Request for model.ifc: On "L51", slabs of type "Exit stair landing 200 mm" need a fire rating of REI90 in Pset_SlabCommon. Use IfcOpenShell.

First a look at what the model holds.

```python
import ifcopenshell
import ifcopenshell.util.element

model = ifcopenshell.open("model.ifc")
print(model.schema)
storey = next(s for s in model.by_type("IfcBuildingStorey") if s.Name == "L51")
slabs = [e for e in ifcopenshell.util.element.get_decomposition(storey) if e.is_a("IfcSlab")]
seen = {}
for e in slabs:
    element_type = ifcopenshell.util.element.get_type(e)
    key = (element_type.Name if element_type != e and element_type else None, ifcopenshell.util.element.get_pset(e, "Pset_SlabCommon", "FireRating"))
    seen[key] = seen.get(key, 0) + 1
for (name, value), count in sorted(seen.items(), key=str):
    print(count, "x", name, "|", value)
```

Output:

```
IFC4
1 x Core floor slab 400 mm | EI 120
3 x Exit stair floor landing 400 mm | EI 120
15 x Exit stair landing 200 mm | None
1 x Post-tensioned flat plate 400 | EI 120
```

```python
import ifcopenshell
import ifcopenshell.api.pset
import ifcopenshell.util.element

model = ifcopenshell.open("model.ifc")

storey = next(s for s in model.by_type("IfcBuildingStorey") if s.Name == "L51")
slabs = [e for e in ifcopenshell.util.element.get_decomposition(storey) if e.is_a("IfcSlab")]

count = 0
for e in slabs:
    element_type = ifcopenshell.util.element.get_type(e)
    if element_type in (None, e) or element_type.Name != "Exit stair landing 200 mm":
        continue
    found = ifcopenshell.util.element.get_pset(e, "Pset_SlabCommon", should_inherit=False)
    if found:
        pset = model.by_id(found["id"])
        if len(ifcopenshell.util.element.get_elements_by_pset(pset)) > 1:
            pset = ifcopenshell.api.pset.unshare_pset(model, products=[e], pset=pset)[0]
    else:
        pset = ifcopenshell.api.pset.add_pset(model, product=e, name="Pset_SlabCommon")
    ifcopenshell.api.pset.edit_pset(model, pset=pset, properties={"FireRating": "REI90"})
    count += 1

print(count, "slabs updated")

model.write("model_updated.ifc")
```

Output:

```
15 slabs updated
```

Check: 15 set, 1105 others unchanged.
